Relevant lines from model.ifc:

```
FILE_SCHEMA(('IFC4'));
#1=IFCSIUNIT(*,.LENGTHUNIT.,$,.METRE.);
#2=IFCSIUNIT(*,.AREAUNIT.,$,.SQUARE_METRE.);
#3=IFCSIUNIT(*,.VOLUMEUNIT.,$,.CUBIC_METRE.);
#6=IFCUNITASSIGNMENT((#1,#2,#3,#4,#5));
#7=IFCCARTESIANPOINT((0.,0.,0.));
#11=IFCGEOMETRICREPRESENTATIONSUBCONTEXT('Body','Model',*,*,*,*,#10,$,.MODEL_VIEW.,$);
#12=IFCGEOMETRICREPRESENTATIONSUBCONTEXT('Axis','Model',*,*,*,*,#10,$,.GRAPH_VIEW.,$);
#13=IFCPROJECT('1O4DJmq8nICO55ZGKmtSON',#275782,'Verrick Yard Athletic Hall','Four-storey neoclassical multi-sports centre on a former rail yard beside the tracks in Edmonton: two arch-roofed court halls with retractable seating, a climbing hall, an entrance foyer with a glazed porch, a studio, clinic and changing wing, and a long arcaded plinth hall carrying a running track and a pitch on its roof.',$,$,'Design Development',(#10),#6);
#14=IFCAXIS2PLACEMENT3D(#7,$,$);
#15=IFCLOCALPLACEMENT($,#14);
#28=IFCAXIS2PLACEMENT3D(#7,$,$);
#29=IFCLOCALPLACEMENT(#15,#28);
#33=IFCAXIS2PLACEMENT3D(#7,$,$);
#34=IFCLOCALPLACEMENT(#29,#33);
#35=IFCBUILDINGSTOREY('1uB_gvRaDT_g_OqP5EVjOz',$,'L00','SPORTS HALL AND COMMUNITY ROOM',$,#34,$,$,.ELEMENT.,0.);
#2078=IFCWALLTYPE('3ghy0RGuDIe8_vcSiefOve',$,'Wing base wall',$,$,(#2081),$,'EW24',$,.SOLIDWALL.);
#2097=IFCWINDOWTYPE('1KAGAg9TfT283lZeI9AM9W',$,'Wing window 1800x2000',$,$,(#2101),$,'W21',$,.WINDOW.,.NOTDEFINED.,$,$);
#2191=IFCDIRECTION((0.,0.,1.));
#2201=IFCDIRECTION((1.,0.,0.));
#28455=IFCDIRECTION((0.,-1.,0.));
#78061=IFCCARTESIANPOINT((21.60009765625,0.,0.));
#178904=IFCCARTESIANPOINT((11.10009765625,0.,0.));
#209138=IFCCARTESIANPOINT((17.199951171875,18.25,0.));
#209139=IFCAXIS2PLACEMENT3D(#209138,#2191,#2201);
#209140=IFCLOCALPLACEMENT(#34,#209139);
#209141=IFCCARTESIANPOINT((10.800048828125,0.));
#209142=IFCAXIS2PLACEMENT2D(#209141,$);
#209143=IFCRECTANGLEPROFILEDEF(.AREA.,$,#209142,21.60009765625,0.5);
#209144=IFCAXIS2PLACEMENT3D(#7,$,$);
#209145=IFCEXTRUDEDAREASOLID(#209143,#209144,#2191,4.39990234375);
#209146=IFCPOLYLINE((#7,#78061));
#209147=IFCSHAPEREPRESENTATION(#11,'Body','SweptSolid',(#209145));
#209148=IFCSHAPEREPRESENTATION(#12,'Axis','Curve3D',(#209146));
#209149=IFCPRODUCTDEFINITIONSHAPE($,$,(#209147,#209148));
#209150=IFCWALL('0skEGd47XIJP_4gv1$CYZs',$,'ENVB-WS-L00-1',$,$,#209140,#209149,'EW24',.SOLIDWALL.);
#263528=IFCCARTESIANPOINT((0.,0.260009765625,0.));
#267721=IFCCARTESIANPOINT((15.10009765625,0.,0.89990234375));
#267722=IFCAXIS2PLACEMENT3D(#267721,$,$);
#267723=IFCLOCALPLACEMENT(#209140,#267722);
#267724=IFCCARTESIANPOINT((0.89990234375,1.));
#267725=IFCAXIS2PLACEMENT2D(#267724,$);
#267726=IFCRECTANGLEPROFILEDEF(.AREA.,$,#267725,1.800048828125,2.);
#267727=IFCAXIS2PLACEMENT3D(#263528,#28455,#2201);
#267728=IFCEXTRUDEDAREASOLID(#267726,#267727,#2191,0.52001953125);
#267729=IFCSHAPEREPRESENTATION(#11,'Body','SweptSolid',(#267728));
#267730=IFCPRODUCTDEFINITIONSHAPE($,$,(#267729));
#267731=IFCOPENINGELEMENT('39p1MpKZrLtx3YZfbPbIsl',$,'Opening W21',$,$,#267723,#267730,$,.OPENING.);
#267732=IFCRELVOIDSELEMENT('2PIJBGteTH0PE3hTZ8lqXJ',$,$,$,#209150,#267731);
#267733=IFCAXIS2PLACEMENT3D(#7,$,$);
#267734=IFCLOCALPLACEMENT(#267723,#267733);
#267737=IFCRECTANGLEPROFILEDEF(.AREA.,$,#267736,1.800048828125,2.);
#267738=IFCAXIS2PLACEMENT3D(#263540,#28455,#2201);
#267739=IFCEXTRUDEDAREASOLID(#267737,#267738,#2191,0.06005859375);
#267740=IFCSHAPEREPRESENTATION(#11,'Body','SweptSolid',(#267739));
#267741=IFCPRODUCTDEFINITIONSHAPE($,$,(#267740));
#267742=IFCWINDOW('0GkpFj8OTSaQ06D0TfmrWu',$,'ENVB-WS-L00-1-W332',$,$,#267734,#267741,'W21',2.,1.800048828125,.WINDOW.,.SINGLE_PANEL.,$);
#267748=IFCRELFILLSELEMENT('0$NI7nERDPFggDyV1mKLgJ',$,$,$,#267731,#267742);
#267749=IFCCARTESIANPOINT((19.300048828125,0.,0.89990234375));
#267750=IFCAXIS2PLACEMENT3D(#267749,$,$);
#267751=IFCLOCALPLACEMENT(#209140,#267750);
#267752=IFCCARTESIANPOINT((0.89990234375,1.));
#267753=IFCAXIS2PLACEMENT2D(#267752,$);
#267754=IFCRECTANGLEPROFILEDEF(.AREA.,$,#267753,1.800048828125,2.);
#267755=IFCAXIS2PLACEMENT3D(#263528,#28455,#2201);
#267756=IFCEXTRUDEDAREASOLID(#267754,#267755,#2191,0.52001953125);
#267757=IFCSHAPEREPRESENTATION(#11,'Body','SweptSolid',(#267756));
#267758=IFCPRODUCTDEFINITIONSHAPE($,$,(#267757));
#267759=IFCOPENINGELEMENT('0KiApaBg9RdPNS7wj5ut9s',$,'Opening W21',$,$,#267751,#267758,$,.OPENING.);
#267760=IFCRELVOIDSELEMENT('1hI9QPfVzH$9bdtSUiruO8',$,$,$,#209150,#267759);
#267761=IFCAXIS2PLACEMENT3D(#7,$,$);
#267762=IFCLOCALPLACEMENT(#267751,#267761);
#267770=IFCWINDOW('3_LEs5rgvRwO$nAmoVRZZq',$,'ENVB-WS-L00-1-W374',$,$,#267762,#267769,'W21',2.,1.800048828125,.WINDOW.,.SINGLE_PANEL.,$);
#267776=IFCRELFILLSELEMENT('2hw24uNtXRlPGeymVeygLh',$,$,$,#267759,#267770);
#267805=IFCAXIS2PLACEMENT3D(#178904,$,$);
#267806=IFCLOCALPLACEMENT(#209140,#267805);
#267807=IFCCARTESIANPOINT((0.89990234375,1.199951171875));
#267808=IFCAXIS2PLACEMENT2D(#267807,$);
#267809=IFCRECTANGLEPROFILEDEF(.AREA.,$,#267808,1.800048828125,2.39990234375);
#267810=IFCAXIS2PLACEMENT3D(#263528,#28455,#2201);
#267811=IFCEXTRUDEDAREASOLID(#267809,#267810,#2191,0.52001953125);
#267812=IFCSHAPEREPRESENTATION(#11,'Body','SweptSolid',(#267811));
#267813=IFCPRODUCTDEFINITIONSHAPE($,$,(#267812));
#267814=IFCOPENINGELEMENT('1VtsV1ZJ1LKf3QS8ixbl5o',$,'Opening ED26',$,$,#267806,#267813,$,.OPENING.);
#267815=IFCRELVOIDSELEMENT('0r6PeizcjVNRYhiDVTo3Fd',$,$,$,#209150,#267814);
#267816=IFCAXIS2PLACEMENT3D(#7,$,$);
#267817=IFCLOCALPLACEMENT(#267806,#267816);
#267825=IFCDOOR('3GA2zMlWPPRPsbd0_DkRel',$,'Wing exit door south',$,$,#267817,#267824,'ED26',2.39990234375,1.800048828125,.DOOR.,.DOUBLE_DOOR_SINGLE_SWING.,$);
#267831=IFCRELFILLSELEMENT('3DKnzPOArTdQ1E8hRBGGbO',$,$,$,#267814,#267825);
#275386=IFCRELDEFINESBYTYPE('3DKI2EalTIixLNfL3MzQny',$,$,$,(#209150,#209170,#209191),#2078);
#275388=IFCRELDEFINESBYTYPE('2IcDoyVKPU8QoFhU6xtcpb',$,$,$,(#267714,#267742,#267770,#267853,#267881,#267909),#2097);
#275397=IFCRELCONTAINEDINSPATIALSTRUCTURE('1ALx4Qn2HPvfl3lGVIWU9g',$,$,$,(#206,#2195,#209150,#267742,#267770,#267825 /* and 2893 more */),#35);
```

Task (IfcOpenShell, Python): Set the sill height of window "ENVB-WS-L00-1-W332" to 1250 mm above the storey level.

```python
import numpy as np
import ifcopenshell
import ifcopenshell.api.geometry
import ifcopenshell.geom
import ifcopenshell.util.element
import ifcopenshell.util.placement
import ifcopenshell.util.shape
import ifcopenshell.util.unit

model = ifcopenshell.open("model.ifc")
unit_scale = ifcopenshell.util.unit.calculate_unit_scale(model)

window = model.by_guid("0GkpFj8OTSaQ06D0TfmrWu")
opening = window.FillsVoids[0].RelatingOpeningElement
storey = ifcopenshell.util.element.get_container(window, ifc_class="IfcBuildingStorey")
level = ifcopenshell.util.placement.get_local_placement(storey.ObjectPlacement)[2, 3]

# The opening's origin need not be at the sill, so measure its lowest point.
shape = ifcopenshell.geom.create_shape(ifcopenshell.geom.settings(), opening)
bottom = ifcopenshell.util.shape.get_shape_bottom_elevation(shape, shape.geometry) / unit_scale
dz = level + 1.25 - bottom

shift = np.array([0.0, 0.0, dz])
# The window is placed relative to its opening, so it follows when the opening moves.
matrix = ifcopenshell.util.placement.get_local_placement(opening.ObjectPlacement)
matrix[:3, 3] += shift
ifcopenshell.api.geometry.edit_object_placement(
    model, product=opening, matrix=matrix, is_si=False, should_transform_children=True
)

print(f"moved by {dz * unit_scale:+.3f} m")

model.write("model-out.ifc")
```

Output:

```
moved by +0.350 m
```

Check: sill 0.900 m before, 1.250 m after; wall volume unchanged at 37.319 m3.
